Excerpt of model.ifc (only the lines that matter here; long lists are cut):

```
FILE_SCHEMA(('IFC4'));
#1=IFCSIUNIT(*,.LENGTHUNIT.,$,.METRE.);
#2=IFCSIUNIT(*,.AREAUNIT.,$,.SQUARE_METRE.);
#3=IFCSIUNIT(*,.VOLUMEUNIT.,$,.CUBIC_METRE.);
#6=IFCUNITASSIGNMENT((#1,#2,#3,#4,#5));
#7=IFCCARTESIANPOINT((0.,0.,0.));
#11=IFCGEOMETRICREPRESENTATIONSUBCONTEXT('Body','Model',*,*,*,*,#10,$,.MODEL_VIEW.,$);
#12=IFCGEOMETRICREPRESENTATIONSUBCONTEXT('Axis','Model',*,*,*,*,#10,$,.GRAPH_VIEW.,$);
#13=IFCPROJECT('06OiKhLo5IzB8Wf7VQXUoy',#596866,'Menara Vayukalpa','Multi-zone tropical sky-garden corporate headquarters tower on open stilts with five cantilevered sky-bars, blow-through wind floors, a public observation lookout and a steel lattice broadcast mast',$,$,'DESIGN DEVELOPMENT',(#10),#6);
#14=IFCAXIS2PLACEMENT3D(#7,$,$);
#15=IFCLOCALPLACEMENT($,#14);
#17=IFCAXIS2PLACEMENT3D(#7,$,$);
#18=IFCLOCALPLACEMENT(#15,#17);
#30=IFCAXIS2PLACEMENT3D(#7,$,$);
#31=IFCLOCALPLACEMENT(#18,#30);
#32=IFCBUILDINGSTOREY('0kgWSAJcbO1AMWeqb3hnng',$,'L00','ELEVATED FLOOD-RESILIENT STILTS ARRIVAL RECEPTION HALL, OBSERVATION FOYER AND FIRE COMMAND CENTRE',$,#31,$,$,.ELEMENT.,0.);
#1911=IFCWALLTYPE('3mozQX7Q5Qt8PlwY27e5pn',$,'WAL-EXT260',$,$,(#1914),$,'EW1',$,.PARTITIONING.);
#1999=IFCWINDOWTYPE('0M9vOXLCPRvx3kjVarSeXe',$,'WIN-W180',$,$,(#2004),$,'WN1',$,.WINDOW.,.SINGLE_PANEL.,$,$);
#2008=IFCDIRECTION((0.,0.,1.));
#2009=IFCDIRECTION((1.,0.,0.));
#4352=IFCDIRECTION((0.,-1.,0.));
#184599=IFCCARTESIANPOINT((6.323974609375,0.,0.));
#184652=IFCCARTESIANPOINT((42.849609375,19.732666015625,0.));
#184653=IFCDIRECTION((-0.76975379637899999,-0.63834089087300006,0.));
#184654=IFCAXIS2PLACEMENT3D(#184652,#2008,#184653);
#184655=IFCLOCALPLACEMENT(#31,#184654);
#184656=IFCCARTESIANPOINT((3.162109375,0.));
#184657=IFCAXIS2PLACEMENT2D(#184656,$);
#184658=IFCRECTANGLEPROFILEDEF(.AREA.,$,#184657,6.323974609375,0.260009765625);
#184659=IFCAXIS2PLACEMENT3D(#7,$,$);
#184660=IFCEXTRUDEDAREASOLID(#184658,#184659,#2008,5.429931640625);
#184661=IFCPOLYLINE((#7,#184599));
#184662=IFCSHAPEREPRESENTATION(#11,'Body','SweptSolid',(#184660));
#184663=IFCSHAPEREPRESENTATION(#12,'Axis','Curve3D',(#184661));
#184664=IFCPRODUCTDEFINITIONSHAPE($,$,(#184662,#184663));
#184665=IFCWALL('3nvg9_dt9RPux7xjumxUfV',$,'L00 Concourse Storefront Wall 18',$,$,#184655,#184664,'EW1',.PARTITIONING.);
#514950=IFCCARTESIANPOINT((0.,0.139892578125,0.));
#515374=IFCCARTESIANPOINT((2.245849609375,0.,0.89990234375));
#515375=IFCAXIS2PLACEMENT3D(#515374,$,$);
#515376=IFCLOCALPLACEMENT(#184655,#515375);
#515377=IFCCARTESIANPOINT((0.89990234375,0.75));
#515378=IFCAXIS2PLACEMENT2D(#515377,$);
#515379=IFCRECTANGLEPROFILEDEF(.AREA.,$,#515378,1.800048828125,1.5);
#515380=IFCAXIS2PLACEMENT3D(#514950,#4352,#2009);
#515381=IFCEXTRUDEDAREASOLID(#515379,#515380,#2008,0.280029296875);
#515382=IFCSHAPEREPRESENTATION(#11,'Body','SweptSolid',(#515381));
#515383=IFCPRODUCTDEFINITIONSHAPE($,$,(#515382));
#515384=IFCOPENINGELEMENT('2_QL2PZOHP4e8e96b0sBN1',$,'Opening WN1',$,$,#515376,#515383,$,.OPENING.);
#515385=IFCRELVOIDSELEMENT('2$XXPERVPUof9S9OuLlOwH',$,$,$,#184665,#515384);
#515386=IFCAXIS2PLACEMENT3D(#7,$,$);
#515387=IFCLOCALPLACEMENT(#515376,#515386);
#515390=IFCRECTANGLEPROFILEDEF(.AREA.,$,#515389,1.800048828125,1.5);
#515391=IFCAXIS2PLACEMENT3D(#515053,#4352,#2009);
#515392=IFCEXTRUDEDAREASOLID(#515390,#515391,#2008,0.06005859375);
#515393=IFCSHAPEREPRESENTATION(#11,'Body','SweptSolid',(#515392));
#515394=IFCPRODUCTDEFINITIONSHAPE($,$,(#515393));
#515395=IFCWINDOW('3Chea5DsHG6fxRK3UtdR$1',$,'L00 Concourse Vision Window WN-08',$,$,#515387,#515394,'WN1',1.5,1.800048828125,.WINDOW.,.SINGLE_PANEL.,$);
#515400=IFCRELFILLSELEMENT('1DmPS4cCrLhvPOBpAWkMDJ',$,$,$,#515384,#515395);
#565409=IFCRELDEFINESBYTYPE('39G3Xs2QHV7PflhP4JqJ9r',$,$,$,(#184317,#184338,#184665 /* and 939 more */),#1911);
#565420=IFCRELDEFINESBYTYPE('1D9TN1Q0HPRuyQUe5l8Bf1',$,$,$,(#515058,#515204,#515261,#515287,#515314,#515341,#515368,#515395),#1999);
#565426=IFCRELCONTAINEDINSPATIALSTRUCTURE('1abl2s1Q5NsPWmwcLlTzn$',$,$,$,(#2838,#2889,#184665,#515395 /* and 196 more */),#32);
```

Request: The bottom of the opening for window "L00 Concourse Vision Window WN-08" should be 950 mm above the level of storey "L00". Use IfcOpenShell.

```python
import numpy as np
import ifcopenshell
import ifcopenshell.api.geometry
import ifcopenshell.geom
import ifcopenshell.util.element
import ifcopenshell.util.placement
import ifcopenshell.util.shape
import ifcopenshell.util.unit

model = ifcopenshell.open("model.ifc")
unit_scale = ifcopenshell.util.unit.calculate_unit_scale(model)

window = model.by_guid("3Chea5DsHG6fxRK3UtdR$1")
opening = window.FillsVoids[0].RelatingOpeningElement
storey = ifcopenshell.util.element.get_container(window, ifc_class="IfcBuildingStorey")
level = ifcopenshell.util.placement.get_local_placement(storey.ObjectPlacement)[2, 3]

# The opening's origin need not be at the sill, so measure its lowest point.
shape = ifcopenshell.geom.create_shape(ifcopenshell.geom.settings(), opening)
bottom = ifcopenshell.util.shape.get_shape_bottom_elevation(shape, shape.geometry) / unit_scale
dz = level + 0.95 / unit_scale - bottom

shift = np.array([0.0, 0.0, dz])
# The window is placed relative to its opening, so it follows when the opening moves.
matrix = ifcopenshell.util.placement.get_local_placement(opening.ObjectPlacement)
matrix[:3, 3] += shift
ifcopenshell.api.geometry.edit_object_placement(
    model, product=opening, matrix=matrix, is_si=False, should_transform_children=True
)

print(f"moved by {dz * unit_scale:+.3f} m")

model.write("model_updated.ifc")
```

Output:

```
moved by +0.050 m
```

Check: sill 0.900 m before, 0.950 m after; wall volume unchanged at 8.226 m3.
